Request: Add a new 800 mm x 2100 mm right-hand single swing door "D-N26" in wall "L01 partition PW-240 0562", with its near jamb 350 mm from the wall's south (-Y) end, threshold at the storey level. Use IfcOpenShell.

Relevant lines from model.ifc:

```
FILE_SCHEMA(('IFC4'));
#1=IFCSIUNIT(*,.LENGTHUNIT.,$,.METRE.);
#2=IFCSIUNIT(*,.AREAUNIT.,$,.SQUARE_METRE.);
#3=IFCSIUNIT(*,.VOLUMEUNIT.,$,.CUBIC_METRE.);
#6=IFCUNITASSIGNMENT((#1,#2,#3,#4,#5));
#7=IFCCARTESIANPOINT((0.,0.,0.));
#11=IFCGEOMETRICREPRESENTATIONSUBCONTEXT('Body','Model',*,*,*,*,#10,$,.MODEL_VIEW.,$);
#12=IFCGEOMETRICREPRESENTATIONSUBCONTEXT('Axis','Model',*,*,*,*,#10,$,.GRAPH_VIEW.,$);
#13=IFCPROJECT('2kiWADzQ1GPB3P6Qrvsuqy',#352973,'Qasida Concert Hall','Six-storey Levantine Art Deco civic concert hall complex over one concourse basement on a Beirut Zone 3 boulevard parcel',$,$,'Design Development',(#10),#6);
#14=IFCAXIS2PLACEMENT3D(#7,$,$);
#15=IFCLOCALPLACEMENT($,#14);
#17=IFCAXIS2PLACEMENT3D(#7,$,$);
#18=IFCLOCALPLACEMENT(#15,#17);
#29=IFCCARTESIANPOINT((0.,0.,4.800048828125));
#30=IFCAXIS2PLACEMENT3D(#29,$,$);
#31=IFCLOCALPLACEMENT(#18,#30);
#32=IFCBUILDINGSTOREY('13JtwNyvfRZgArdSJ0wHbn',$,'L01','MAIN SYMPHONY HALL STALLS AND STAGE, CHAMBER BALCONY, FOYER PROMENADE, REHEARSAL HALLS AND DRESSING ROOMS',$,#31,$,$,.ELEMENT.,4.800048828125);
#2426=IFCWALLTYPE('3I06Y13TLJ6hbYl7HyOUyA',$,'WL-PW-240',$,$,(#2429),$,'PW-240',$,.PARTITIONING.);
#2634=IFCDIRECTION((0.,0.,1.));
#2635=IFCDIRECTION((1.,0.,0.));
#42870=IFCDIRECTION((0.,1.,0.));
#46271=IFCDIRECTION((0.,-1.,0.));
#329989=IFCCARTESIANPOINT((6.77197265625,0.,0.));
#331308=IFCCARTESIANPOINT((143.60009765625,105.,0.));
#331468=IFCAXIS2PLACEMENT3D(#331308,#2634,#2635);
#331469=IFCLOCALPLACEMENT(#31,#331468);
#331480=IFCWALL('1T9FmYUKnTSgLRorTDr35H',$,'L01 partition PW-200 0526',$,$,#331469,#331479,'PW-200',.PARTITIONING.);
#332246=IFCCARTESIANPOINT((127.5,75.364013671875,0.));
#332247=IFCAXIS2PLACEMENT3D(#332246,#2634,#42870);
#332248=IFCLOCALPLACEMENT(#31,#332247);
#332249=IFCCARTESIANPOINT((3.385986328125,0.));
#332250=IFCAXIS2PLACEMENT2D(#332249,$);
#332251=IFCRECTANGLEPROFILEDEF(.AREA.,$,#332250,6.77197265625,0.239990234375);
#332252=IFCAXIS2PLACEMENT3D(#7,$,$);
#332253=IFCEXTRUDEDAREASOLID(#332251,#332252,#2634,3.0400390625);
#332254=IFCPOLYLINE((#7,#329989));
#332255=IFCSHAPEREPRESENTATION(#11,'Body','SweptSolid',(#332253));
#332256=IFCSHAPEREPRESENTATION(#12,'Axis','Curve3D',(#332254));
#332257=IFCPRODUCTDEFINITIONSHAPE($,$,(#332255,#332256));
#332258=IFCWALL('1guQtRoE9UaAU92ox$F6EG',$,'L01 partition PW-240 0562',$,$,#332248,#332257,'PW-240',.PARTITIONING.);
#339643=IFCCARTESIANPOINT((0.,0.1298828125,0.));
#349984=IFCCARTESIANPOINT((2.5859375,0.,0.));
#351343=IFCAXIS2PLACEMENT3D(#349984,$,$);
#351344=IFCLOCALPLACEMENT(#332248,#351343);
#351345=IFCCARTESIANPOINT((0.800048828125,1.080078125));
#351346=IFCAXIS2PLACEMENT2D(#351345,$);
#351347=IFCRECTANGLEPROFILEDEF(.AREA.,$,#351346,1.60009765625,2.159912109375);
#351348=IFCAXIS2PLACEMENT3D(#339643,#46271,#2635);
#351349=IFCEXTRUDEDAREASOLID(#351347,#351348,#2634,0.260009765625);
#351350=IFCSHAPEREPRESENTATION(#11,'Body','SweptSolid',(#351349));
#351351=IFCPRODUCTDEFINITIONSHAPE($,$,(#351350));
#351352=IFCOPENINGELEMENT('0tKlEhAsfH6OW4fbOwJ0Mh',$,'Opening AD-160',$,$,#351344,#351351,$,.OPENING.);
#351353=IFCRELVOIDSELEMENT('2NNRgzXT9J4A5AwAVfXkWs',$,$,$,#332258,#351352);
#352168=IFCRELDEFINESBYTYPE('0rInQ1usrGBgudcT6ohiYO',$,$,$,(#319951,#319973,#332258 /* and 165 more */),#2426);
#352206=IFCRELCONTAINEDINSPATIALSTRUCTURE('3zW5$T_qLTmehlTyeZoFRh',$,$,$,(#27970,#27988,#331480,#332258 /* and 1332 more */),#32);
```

```python
import numpy as np
import ifcopenshell
import ifcopenshell.api.feature
import ifcopenshell.api.geometry
import ifcopenshell.api.root
import ifcopenshell.api.spatial
import ifcopenshell.geom
import ifcopenshell.util.element
import ifcopenshell.util.placement
import ifcopenshell.util.representation
import ifcopenshell.util.shape
import ifcopenshell.util.unit

model = ifcopenshell.open("model.ifc")
unit_scale = ifcopenshell.util.unit.calculate_unit_scale(model)
settings = ifcopenshell.geom.settings()


def volume(element):
    """Net volume in cubic metres, openings subtracted."""
    shape = ifcopenshell.geom.create_shape(settings, element)
    return ifcopenshell.util.shape.get_volume(shape.geometry)


wall = model.by_guid("1guQtRoE9UaAU92ox$F6EG")
storey = ifcopenshell.util.element.get_container(wall, ifc_class="IfcBuildingStorey")
context = ifcopenshell.util.representation.get_context(model, "Model", "Body", "MODEL_VIEW")
before = volume(wall)

width, height, from_end, sill = 0.8, 2.1, 0.35, 0.0  # metres

# The wall runs along its own X axis, and the end named is its -X end.
wall_shape = ifcopenshell.geom.create_shape(settings, wall)
x, y, z = ifcopenshell.util.shape.get_vertices(wall_shape.geometry).T
start = x.min() + from_end
face, thickness = float(y.min()), float(y.max() - y.min())
wall_matrix = ifcopenshell.util.placement.get_local_placement(wall.ObjectPlacement)
level = ifcopenshell.util.placement.get_local_placement(storey.ObjectPlacement)[2, 3]


def in_wall(x, y):
    """Placement at x, y metres in the wall's axes, at sill height."""
    matrix = wall_matrix.copy()
    matrix[:, 3] = wall_matrix @ np.array([x / unit_scale, y / unit_scale, 0.0, 1.0])
    matrix[2, 3] = level + sill / unit_scale
    return matrix


# Opening: a box that overshoots both wall faces by 50 mm.
opening = ifcopenshell.api.root.create_entity(model, ifc_class="IfcOpeningElement", predefined_type="OPENING")
box = ifcopenshell.api.geometry.add_wall_representation(
    model, context=context, length=width, height=height, thickness=thickness + 0.1
)
ifcopenshell.api.geometry.assign_representation(model, product=opening, representation=box)
ifcopenshell.api.geometry.edit_object_placement(model, product=opening, matrix=in_wall(start, face - 0.05), is_si=False)
ifcopenshell.api.feature.add_feature(model, feature=opening, element=wall)

door = ifcopenshell.api.root.create_entity(model, ifc_class="IfcDoor", name="D-N26", predefined_type="DOOR")
door.OverallWidth, door.OverallHeight = width / unit_scale, height / unit_scale
door.OperationType = "SINGLE_SWING_RIGHT"
body = ifcopenshell.api.geometry.add_door_representation(
    model,
    context=context,
    overall_width=door.OverallWidth,
    overall_height=door.OverallHeight,
    operation_type="SINGLE_SWING_RIGHT",
    lining_properties={"LiningDepth": thickness / unit_scale, "ThresholdDepth": thickness / unit_scale},
)
ifcopenshell.api.geometry.assign_representation(model, product=door, representation=body)
ifcopenshell.api.spatial.assign_container(model, products=[door], relating_structure=storey)
ifcopenshell.api.feature.add_filling(model, opening=opening, element=door)

# The lining spans the wall, so the door starts at the wall face.
ifcopenshell.api.geometry.edit_object_placement(model, product=door, matrix=in_wall(start, face), is_si=False)

after = volume(wall)

print(f"wall volume {before:.3f} -> {after:.3f} m3")

model.write("model-out.ifc")
```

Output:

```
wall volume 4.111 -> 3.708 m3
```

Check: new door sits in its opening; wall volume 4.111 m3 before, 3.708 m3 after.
